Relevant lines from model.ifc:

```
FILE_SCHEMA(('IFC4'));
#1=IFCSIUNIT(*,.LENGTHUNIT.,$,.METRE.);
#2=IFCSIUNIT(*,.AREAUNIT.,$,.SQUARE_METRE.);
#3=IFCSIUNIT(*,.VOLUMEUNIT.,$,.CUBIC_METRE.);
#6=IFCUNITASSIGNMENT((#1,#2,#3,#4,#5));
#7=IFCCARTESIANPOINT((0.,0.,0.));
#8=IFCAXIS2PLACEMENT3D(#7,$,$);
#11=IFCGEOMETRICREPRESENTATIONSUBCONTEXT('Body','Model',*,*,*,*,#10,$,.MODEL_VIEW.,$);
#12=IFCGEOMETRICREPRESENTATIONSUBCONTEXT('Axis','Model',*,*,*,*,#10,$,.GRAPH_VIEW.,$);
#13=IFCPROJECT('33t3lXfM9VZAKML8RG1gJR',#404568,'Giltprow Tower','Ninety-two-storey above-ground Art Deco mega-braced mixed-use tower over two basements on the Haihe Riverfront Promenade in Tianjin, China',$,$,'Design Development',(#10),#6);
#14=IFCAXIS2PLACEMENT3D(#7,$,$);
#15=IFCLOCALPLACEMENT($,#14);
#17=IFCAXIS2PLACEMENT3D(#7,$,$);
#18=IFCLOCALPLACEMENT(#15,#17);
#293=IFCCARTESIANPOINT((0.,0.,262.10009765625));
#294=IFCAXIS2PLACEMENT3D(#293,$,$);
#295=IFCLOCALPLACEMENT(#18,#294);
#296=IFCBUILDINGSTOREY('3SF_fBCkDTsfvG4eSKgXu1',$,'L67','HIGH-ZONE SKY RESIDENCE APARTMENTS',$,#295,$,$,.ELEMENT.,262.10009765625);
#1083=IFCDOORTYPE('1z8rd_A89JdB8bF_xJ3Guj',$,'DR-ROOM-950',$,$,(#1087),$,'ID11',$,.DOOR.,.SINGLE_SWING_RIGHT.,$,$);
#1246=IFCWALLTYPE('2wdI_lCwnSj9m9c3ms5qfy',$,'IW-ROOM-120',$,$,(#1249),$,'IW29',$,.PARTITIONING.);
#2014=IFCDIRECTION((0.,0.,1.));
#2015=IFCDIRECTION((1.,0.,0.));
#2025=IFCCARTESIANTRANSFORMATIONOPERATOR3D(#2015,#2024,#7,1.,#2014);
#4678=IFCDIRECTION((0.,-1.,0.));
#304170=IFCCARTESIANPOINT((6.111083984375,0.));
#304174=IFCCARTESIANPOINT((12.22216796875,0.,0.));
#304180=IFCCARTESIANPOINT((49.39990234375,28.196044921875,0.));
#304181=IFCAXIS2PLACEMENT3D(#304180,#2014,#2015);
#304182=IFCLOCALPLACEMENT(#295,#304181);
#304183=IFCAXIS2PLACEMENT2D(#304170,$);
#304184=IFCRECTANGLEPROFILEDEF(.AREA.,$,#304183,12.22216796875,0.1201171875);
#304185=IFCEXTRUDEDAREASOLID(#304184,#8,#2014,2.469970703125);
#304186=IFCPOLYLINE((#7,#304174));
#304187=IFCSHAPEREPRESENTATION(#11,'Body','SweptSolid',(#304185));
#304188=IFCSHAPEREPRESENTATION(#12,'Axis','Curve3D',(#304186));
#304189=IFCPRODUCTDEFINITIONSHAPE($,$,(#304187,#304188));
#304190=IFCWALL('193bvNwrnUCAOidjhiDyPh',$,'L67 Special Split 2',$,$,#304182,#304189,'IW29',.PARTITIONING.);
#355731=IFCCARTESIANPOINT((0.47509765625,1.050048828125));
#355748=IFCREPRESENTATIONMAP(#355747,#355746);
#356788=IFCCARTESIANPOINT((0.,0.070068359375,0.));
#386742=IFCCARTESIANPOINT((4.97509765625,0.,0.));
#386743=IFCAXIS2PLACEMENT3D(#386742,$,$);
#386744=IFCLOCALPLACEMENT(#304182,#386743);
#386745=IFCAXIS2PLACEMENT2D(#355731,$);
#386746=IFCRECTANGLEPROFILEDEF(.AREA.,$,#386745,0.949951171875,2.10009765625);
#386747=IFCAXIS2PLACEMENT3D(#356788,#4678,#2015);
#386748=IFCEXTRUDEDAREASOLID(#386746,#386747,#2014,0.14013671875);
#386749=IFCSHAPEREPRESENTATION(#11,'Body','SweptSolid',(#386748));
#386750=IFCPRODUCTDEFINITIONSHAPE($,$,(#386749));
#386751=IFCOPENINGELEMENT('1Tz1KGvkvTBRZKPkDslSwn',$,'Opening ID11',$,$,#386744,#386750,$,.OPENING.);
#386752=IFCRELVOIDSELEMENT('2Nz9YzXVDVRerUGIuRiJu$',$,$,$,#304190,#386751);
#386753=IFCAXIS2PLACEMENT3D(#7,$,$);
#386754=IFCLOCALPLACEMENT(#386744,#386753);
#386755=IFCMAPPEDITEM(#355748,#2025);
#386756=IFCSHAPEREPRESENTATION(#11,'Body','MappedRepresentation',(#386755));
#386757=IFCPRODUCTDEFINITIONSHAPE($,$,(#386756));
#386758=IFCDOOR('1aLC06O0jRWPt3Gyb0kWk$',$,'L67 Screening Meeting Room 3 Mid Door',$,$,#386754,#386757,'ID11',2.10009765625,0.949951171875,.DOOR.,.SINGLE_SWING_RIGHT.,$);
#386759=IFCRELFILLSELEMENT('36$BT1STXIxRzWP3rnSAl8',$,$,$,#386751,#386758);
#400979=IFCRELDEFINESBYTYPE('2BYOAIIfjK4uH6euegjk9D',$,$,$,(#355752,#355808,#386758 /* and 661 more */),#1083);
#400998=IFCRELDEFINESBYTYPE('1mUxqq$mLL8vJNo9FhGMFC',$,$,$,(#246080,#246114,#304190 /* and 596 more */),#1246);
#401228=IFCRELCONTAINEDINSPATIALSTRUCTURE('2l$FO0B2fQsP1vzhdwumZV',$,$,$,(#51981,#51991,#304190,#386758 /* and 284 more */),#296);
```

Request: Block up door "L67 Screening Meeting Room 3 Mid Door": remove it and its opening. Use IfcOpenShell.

```python
import ifcopenshell
import ifcopenshell.api.feature
import ifcopenshell.api.root
import ifcopenshell.geom
import ifcopenshell.util.shape

model = ifcopenshell.open("model.ifc")
settings = ifcopenshell.geom.settings()


def volume(element):
    """Net volume in cubic metres, openings subtracted."""
    shape = ifcopenshell.geom.create_shape(settings, element)
    return ifcopenshell.util.shape.get_volume(shape.geometry)


door = model.by_guid("1aLC06O0jRWPt3Gyb0kWk$")
opening = door.FillsVoids[0].RelatingOpeningElement
wall = opening.VoidsElements[0].RelatingBuildingElement
before = volume(wall)

ifcopenshell.api.root.remove_product(model, product=door)
ifcopenshell.api.feature.remove_feature(model, feature=opening)

after = volume(wall)

print(f"wall volume {before:.3f} -> {after:.3f} m3")

model.write("model_edited.ifc")
```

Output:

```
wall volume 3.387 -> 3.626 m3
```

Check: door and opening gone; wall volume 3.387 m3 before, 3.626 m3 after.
